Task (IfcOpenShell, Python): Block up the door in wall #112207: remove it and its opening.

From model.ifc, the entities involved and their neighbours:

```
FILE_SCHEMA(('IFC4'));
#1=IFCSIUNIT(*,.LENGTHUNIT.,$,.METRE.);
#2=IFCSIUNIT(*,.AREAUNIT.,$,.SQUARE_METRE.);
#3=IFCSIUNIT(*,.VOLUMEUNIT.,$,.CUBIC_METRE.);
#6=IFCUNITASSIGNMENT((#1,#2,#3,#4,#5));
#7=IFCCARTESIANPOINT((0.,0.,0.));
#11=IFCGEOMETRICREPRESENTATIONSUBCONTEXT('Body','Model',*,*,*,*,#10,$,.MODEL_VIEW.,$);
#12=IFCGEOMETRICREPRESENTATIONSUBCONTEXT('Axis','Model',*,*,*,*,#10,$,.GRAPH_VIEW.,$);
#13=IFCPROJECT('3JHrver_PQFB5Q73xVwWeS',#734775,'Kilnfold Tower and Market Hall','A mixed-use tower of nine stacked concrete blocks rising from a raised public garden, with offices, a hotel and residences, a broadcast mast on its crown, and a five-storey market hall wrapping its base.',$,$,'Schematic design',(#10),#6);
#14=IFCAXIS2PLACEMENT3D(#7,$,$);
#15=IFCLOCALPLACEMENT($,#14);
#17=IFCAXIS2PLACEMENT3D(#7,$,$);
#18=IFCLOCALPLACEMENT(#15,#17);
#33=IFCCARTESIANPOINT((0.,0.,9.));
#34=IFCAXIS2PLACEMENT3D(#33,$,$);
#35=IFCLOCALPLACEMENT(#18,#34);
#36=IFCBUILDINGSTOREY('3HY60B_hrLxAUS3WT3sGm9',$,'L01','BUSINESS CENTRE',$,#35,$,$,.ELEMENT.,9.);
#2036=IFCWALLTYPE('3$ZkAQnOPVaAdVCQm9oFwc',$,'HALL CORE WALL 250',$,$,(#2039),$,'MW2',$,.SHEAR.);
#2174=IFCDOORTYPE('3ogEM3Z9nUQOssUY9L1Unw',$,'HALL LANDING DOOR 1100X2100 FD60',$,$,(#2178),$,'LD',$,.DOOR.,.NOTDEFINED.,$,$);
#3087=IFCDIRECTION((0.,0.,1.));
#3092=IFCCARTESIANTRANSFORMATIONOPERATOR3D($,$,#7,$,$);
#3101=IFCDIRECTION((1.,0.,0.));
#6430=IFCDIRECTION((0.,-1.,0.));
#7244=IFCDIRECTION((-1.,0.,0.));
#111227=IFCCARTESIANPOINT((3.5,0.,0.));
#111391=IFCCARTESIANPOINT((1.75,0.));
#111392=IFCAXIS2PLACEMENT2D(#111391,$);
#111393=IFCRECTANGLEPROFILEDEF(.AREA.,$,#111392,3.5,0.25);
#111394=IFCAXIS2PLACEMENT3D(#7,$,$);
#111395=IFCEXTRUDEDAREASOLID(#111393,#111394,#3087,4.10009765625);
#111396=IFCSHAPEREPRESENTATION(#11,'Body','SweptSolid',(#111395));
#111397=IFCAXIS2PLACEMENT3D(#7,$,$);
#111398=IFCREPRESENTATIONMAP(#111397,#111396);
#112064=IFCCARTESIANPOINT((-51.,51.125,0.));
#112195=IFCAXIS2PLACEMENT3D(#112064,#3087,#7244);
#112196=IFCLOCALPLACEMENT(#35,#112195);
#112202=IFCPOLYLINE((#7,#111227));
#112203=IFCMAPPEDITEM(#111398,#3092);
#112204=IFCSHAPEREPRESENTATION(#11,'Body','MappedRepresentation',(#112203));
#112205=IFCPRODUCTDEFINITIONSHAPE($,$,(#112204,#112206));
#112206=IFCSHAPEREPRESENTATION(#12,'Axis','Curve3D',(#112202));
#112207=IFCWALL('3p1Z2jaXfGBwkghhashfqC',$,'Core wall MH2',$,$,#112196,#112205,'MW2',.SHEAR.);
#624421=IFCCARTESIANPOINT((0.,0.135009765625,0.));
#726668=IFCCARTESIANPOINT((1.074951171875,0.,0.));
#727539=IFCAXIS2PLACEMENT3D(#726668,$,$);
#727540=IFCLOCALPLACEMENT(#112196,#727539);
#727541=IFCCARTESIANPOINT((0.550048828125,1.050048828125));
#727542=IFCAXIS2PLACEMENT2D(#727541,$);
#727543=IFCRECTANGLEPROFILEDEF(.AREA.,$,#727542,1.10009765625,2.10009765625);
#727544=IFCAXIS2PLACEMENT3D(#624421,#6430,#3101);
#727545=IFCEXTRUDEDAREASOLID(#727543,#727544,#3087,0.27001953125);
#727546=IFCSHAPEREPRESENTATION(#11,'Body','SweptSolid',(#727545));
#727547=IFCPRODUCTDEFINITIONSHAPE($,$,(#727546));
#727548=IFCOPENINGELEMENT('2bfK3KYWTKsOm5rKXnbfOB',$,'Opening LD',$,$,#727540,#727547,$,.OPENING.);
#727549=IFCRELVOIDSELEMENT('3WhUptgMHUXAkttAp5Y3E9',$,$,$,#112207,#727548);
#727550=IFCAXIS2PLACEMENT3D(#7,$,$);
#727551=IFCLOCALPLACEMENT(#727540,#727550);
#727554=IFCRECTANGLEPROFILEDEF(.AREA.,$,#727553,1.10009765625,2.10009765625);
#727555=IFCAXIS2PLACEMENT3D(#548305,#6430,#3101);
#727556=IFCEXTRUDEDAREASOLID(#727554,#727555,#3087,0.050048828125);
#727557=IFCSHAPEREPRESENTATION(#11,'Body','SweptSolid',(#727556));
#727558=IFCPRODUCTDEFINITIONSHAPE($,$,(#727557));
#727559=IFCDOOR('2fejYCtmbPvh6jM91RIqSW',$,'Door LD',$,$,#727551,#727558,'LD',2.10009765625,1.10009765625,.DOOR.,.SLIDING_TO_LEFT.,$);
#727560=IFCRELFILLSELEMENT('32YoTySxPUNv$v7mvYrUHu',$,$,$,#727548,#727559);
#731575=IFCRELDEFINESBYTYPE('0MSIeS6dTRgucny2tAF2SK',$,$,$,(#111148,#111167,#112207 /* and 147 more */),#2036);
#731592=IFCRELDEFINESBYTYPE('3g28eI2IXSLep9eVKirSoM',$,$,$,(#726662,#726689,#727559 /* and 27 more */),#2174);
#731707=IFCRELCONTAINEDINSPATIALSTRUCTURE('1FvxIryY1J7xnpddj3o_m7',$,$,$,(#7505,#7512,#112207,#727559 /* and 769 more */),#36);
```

```python
import ifcopenshell
import ifcopenshell.api.feature
import ifcopenshell.api.root
import ifcopenshell.geom
import ifcopenshell.util.shape

model = ifcopenshell.open("model.ifc")
settings = ifcopenshell.geom.settings()


def volume(element):
    """Net volume in cubic metres, openings subtracted."""
    shape = ifcopenshell.geom.create_shape(settings, element)
    return ifcopenshell.util.shape.get_volume(shape.geometry)


door = model.by_guid("2fejYCtmbPvh6jM91RIqSW")
opening = door.FillsVoids[0].RelatingOpeningElement
wall = opening.VoidsElements[0].RelatingBuildingElement
before = volume(wall)

ifcopenshell.api.root.remove_product(model, product=door)
ifcopenshell.api.feature.remove_feature(model, feature=opening)

after = volume(wall)

print(f"wall volume {before:.3f} -> {after:.3f} m3")

model.write("model_v2.ifc")
```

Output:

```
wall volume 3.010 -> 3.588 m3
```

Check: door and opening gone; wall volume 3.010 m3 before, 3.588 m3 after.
